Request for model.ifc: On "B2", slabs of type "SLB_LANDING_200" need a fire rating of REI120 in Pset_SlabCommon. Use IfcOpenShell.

First a look at what the model holds.

```python
import ifcopenshell
import ifcopenshell.util.element

model = ifcopenshell.open("model.ifc")
print(model.schema)
storey = next(s for s in model.by_type("IfcBuildingStorey") if s.Name == "B2")
slabs = [e for e in ifcopenshell.util.element.get_decomposition(storey) if e.is_a("IfcSlab")]
seen = {}
for e in slabs:
    element_type = ifcopenshell.util.element.get_type(e)
    key = (element_type.Name if element_type != e and element_type else None, ifcopenshell.util.element.get_pset(e, "Pset_SlabCommon", "FireRating"))
    seen[key] = seen.get(key, 0) + 1
for (name, value), count in sorted(seen.items(), key=str):
    print(count, "x", name, "|", value)
```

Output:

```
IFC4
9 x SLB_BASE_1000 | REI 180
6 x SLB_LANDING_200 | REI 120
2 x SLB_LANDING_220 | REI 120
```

```python
import ifcopenshell
import ifcopenshell.api.pset
import ifcopenshell.util.element

model = ifcopenshell.open("model.ifc")

storey = next(s for s in model.by_type("IfcBuildingStorey") if s.Name == "B2")
slabs = [e for e in ifcopenshell.util.element.get_decomposition(storey) if e.is_a("IfcSlab")]

count = 0
for e in slabs:
    element_type = ifcopenshell.util.element.get_type(e)
    if element_type in (None, e) or element_type.Name != "SLB_LANDING_200":
        continue
    # add_pset returns the element's existing set when there is one.
    pset = ifcopenshell.api.pset.add_pset(model, product=e, name="Pset_SlabCommon")
    ifcopenshell.api.pset.edit_pset(model, pset=pset, properties={"FireRating": "REI120"})
    count += 1

print(count, "slabs updated")

model.write("model_edited.ifc")
```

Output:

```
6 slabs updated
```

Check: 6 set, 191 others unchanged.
